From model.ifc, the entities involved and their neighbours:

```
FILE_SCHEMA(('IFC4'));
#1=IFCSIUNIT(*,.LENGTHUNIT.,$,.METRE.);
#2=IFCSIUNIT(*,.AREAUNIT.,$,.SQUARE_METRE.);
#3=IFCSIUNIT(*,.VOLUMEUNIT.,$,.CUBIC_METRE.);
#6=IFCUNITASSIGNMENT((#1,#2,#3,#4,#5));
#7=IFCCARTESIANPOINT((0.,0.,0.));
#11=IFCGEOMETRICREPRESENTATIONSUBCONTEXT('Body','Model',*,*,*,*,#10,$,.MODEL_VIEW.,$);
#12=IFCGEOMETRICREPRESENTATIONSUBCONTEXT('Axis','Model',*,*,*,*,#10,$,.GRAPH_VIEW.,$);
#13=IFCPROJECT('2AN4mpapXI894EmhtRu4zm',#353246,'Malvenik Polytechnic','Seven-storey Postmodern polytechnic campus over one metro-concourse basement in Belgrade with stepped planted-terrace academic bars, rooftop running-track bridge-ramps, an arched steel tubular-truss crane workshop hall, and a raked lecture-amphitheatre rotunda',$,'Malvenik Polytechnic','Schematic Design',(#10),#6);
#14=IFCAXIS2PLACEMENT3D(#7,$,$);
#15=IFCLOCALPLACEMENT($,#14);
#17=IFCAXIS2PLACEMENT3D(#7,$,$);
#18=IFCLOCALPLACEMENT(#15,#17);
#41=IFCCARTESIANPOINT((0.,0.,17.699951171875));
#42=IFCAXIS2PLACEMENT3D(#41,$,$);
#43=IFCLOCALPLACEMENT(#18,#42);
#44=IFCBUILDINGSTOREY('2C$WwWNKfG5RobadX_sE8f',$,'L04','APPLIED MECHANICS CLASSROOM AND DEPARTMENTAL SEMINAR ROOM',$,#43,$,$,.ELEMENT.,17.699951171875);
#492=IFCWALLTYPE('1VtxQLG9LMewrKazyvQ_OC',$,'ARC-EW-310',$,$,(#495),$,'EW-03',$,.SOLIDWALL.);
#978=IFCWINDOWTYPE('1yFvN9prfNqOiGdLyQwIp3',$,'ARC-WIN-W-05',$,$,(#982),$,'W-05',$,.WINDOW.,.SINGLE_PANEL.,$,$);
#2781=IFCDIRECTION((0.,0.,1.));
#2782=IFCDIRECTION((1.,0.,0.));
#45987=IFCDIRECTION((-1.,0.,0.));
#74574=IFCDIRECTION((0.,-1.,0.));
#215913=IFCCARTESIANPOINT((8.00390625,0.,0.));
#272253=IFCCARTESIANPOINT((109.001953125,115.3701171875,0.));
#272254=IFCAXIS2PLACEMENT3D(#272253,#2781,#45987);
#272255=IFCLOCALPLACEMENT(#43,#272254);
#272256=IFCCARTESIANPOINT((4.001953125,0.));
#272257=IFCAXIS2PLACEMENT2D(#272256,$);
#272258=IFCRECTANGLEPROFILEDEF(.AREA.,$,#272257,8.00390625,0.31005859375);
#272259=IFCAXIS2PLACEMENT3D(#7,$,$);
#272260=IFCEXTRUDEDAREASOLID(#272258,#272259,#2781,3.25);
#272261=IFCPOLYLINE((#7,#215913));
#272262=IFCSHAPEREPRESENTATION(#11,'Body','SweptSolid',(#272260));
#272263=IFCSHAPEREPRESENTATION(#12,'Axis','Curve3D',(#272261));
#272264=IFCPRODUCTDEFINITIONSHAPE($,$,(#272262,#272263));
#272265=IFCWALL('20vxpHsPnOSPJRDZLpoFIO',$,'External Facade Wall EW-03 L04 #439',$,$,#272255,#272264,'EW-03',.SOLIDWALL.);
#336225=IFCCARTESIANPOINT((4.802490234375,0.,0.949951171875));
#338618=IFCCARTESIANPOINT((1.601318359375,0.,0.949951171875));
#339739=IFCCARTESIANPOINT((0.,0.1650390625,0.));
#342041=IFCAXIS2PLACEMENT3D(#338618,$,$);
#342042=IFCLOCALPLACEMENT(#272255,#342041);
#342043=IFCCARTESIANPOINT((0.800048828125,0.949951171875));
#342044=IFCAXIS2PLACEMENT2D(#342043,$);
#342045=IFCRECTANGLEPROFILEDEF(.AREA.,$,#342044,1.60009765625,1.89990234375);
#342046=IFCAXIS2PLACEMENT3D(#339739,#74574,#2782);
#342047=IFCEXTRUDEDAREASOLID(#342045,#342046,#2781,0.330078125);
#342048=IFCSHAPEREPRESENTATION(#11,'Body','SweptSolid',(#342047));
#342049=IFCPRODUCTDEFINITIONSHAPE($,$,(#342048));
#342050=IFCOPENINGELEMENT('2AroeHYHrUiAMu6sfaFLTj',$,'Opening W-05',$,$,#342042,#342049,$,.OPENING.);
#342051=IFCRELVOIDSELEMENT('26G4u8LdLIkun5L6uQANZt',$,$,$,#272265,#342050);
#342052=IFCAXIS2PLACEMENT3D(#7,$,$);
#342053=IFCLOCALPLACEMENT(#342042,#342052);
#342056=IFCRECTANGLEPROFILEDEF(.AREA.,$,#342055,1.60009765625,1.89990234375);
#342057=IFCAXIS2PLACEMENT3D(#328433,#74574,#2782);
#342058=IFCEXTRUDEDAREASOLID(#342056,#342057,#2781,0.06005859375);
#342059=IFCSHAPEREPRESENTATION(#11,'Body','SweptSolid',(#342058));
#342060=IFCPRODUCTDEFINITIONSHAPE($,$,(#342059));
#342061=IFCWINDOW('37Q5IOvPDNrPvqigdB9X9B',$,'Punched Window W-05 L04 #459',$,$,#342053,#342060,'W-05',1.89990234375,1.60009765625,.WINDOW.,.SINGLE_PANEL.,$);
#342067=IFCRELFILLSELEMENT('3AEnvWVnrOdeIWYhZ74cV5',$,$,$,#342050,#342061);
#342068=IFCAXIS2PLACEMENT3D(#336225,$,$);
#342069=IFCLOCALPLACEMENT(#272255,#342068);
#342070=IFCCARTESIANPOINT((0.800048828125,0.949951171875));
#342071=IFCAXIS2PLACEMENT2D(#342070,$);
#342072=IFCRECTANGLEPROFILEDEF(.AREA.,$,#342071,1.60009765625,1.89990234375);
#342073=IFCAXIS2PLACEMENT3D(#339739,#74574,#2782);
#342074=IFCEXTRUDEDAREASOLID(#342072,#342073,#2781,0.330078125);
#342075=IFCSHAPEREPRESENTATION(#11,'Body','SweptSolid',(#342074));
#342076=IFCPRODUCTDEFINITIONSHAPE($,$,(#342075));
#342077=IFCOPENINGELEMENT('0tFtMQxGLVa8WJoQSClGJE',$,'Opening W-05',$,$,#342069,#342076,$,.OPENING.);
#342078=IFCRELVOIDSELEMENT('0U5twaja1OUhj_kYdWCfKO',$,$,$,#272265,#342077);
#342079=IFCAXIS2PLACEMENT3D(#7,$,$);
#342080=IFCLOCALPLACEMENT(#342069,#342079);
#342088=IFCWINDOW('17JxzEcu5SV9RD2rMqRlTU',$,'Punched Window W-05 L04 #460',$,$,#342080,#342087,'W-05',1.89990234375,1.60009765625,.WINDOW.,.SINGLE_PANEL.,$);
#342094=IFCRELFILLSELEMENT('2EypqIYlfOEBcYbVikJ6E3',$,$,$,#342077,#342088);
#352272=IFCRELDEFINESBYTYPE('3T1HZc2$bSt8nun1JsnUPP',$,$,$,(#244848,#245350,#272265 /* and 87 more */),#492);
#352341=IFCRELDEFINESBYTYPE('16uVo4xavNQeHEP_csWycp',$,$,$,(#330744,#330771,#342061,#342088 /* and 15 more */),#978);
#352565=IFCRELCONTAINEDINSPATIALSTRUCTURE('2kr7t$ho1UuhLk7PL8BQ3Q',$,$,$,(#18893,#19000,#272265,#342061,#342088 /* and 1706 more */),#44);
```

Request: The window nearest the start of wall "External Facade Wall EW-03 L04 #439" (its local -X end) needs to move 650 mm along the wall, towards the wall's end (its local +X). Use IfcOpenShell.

```python
import ifcopenshell
import ifcopenshell.api.geometry
import ifcopenshell.util.placement
import ifcopenshell.util.unit

model = ifcopenshell.open("model.ifc")
unit_scale = ifcopenshell.util.unit.calculate_unit_scale(model)

window = model.by_id(342061)
opening = window.FillsVoids[0].RelatingOpeningElement
wall = opening.VoidsElements[0].RelatingBuildingElement

wall_matrix = ifcopenshell.util.placement.get_local_placement(wall.ObjectPlacement)
shift = wall_matrix[:3, 0] * 0.65 / unit_scale
before = ifcopenshell.util.placement.get_local_placement(window.ObjectPlacement)[:3, 3].copy()

# The window is placed relative to its opening, so it follows when the opening moves.
matrix = ifcopenshell.util.placement.get_local_placement(opening.ObjectPlacement)
matrix[:3, 3] += shift
ifcopenshell.api.geometry.edit_object_placement(
    model, product=opening, matrix=matrix, is_si=False, should_transform_children=True
)

after = ifcopenshell.util.placement.get_local_placement(window.ObjectPlacement)[:3, 3]
print("window moved by", (after - before).round(3) + 0.0)

model.write("model_v2.ifc")
```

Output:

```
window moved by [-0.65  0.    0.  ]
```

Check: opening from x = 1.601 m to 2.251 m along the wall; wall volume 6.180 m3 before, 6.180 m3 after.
